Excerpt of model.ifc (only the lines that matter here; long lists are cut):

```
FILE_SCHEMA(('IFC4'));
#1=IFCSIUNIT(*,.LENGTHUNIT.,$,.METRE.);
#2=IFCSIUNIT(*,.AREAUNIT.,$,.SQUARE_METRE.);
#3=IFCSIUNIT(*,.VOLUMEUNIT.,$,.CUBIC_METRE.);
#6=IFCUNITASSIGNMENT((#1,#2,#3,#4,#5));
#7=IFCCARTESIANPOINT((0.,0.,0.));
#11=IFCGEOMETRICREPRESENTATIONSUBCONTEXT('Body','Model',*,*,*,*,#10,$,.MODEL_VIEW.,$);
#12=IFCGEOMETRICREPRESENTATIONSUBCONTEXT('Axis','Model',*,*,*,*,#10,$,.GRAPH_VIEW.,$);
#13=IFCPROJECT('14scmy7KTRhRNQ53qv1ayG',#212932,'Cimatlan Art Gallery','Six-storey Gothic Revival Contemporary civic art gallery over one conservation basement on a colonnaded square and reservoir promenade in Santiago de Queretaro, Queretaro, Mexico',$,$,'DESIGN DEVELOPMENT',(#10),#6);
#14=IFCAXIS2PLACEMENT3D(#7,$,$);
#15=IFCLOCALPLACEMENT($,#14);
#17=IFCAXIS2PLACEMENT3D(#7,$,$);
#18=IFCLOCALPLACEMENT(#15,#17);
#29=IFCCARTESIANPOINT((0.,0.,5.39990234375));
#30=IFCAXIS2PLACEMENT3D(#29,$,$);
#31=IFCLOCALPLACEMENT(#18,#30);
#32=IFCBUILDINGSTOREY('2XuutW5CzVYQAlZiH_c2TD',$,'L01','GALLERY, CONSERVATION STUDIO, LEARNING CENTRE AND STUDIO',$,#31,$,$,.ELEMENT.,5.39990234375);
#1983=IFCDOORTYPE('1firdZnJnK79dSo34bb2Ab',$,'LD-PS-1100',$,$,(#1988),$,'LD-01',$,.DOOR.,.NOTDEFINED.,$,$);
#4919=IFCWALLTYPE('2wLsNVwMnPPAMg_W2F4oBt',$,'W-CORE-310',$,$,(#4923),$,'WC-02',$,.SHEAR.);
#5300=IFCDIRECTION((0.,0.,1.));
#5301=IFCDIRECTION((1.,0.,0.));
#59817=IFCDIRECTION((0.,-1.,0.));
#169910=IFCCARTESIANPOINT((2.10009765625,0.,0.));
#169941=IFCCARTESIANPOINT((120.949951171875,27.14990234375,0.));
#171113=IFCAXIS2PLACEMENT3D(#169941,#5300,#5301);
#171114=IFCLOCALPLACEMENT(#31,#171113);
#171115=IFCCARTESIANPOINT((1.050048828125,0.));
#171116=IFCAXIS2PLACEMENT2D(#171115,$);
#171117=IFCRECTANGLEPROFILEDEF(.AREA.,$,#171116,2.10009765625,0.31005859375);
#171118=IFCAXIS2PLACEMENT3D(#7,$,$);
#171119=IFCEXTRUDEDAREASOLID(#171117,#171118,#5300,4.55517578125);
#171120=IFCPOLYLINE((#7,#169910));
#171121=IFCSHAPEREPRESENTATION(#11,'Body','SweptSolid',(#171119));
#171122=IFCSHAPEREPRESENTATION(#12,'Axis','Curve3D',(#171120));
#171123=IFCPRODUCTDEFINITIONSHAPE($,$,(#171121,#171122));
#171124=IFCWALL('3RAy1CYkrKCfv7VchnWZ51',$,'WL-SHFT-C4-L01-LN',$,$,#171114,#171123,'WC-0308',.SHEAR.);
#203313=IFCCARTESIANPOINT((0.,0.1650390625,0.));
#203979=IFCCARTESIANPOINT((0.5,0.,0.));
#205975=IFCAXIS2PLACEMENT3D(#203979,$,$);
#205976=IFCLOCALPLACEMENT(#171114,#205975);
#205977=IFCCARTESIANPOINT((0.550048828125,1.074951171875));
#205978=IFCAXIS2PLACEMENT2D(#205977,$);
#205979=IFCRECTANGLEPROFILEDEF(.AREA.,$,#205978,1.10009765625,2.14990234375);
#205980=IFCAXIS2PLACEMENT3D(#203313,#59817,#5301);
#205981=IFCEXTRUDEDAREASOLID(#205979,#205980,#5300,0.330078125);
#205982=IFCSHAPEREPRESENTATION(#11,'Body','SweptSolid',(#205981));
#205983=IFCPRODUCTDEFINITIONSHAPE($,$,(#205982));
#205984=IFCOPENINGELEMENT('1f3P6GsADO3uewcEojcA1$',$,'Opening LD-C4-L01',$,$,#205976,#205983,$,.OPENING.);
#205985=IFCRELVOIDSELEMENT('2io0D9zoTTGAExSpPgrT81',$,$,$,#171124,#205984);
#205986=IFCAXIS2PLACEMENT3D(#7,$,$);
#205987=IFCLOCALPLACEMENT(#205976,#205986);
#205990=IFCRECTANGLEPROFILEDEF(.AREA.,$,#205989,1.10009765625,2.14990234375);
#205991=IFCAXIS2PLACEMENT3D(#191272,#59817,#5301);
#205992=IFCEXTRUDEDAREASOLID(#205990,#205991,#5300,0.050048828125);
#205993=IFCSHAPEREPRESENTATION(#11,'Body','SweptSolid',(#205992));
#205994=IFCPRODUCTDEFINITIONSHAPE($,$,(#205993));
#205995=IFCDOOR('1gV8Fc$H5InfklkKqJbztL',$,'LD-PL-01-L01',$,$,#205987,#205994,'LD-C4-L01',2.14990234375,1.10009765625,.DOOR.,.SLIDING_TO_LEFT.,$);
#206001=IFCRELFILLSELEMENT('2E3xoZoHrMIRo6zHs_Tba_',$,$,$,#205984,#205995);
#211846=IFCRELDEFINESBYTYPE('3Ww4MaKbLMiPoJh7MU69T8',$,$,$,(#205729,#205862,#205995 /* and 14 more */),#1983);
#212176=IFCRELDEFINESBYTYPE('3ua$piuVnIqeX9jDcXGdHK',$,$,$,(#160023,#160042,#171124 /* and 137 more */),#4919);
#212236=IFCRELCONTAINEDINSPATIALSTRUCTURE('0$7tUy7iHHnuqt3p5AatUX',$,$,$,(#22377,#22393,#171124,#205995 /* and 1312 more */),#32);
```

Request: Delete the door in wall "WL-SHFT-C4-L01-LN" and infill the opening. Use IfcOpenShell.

```python
import ifcopenshell
import ifcopenshell.api.feature
import ifcopenshell.api.root
import ifcopenshell.geom
import ifcopenshell.util.shape

model = ifcopenshell.open("model.ifc")
settings = ifcopenshell.geom.settings()


def volume(element):
    """Net volume in cubic metres, openings subtracted."""
    shape = ifcopenshell.geom.create_shape(settings, element)
    return ifcopenshell.util.shape.get_volume(shape.geometry)


door = model.by_guid("1gV8Fc$H5InfklkKqJbztL")
opening = door.FillsVoids[0].RelatingOpeningElement
wall = opening.VoidsElements[0].RelatingBuildingElement
before = volume(wall)

ifcopenshell.api.root.remove_product(model, product=door)
ifcopenshell.api.feature.remove_feature(model, feature=opening)

after = volume(wall)

print(f"wall volume {before:.3f} -> {after:.3f} m3")

model.write("model_rev.ifc")
```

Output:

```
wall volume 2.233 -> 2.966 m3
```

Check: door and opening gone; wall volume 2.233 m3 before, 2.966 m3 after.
